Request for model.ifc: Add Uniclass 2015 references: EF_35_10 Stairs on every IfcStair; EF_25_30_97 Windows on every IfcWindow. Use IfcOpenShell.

First a look at what the model holds.

```python
import ifcopenshell

model = ifcopenshell.open("model.ifc")
print(model.schema)
print("classifications:", [c.Name for c in model.by_type("IfcClassification")])
for ifc_class in ("IfcDoor", "IfcRoof", "IfcStair", "IfcWall", "IfcWindow"):
    print(ifc_class, len(model.by_type(ifc_class)))
```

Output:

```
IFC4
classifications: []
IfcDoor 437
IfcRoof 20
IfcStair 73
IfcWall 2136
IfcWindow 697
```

```python
import ifcopenshell
import ifcopenshell.api.classification

model = ifcopenshell.open("model.ifc")

system = ifcopenshell.api.classification.add_classification(model, classification="Uniclass 2015")

codes = {
    "IfcStair": ("EF_35_10", "Stairs"),
    "IfcWindow": ("EF_25_30_97", "Windows"),
}
for ifc_class, (code, name) in codes.items():
    products = model.by_type(ifc_class)
    ifcopenshell.api.classification.add_reference(
        model, products=products, classification=system, identification=code, name=name
    )
    print(code, len(products))

model.write("model_rev.ifc")
```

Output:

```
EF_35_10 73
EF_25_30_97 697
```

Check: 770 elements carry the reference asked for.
